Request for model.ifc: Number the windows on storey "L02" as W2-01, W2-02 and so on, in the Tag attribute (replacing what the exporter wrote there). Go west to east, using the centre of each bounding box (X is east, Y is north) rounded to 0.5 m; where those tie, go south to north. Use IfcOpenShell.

First a look at what the model holds.

```python
import ifcopenshell
import ifcopenshell.util.element
import ifcopenshell.util.placement

model = ifcopenshell.open("model.ifc")
print(model.schema)
storey = next(s for s in model.by_type("IfcBuildingStorey") if s.Name == "L02")
windows = [e for e in ifcopenshell.util.element.get_decomposition(storey) if e.is_a("IfcWindow")]
for e in sorted(windows, key=lambda e: e.id()):
    origin = ifcopenshell.util.placement.get_local_placement(e.ObjectPlacement)[:3, 3]
    print(e.id(), e.Tag, e.Name, origin.round(2) + 0.0, sep=" | ")
```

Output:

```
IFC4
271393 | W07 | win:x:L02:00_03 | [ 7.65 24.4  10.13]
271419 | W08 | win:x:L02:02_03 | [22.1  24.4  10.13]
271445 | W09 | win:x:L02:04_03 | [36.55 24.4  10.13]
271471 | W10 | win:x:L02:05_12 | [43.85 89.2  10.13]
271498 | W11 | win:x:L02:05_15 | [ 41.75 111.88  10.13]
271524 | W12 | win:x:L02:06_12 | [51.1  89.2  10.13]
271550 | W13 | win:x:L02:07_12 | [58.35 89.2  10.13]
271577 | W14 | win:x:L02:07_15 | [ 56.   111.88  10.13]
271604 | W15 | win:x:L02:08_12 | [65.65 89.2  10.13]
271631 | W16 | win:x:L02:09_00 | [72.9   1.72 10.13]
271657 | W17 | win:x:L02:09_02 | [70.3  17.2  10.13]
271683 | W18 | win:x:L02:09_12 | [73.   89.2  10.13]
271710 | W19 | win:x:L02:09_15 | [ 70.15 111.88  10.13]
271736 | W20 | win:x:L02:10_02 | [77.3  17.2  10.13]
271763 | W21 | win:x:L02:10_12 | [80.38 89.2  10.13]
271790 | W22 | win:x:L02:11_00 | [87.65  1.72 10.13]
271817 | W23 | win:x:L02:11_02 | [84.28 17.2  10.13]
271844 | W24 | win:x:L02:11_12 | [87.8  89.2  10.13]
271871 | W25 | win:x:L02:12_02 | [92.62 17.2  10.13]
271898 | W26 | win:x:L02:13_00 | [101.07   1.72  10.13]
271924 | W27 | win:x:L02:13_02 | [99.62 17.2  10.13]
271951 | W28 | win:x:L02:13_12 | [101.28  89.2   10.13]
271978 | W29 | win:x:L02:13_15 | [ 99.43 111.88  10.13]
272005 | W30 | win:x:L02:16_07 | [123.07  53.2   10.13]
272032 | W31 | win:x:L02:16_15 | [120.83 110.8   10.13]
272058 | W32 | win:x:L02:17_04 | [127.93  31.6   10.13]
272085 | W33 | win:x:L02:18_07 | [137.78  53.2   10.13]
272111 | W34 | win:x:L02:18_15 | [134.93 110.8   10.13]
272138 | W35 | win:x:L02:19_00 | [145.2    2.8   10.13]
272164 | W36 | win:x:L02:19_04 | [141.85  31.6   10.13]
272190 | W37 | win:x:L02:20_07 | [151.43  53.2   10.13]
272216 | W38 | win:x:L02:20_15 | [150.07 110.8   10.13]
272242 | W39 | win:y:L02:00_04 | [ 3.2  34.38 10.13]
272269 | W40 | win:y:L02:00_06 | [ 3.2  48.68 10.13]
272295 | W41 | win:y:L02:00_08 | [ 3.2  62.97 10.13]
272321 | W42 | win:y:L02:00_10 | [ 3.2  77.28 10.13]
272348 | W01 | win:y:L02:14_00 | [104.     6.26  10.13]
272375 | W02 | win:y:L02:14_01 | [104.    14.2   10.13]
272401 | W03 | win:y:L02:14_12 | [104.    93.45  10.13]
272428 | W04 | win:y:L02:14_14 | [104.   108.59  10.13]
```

```python
import ifcopenshell
import ifcopenshell.geom
import ifcopenshell.util.element
import ifcopenshell.util.shape

model = ifcopenshell.open("model.ifc")
settings = ifcopenshell.geom.settings()
settings.set("use-world-coords", True)


def centre(element):
    shape = ifcopenshell.geom.create_shape(settings, element)
    return ifcopenshell.util.shape.get_bbox_centroid(shape.geometry)


storey = next(s for s in model.by_type("IfcBuildingStorey") if s.Name == "L02")
windows = [e for e in ifcopenshell.util.element.get_decomposition(storey) if e.is_a("IfcWindow")]

# Insertion points can sit at a corner or the storey origin, so sort by the geometry (in metres).
centres = {e: centre(e) for e in windows}
windows.sort(key=lambda e: (round(centres[e][0] / 0.5), centres[e][1]))

for i, e in enumerate(windows, start=1):
    number = f"W2-{i:02d}"
    e.Tag = number
    print(e.id(), number)

model.write("model_rev.ifc")
```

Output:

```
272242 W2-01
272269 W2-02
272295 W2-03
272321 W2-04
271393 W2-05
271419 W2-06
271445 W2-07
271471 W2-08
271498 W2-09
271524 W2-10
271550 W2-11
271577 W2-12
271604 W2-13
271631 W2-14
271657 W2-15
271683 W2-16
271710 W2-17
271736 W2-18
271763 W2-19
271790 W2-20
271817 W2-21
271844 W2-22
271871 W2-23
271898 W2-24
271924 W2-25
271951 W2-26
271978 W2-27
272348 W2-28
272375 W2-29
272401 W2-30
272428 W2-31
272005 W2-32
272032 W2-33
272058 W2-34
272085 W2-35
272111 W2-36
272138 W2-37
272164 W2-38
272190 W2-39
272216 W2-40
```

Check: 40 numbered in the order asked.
